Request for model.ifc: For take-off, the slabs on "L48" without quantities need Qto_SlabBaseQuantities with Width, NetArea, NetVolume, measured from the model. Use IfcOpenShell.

First a look at what the model holds.

```python
import ifcopenshell
import ifcopenshell.util.element
import ifcopenshell.util.unit

model = ifcopenshell.open("model.ifc")
print(model.schema)
for unit_type in ("LENGTHUNIT", "AREAUNIT", "VOLUMEUNIT"):
    print(unit_type, ifcopenshell.util.unit.calculate_unit_scale(model, unit_type))
storey = next(s for s in model.by_type("IfcBuildingStorey") if s.Name == "L48")
slabs = [e for e in ifcopenshell.util.element.get_decomposition(storey) if e.is_a("IfcSlab")]
for e in sorted(slabs, key=lambda e: e.id()):
    print(e.id(), e.is_a(), e.Name, list(ifcopenshell.util.element.get_psets(e, qtos_only=True)), sep=" | ")
```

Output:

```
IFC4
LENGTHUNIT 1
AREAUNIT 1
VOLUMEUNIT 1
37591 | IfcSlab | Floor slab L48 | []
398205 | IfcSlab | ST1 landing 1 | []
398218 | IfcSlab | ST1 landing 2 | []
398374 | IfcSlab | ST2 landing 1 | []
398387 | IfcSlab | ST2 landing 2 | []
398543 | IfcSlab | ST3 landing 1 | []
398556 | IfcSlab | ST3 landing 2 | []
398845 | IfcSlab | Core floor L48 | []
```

```python
import ifcopenshell
import ifcopenshell.api.pset
import ifcopenshell.geom
import ifcopenshell.util.element
import ifcopenshell.util.shape
import ifcopenshell.util.unit

model = ifcopenshell.open("model.ifc")
unit_scale = ifcopenshell.util.unit.calculate_unit_scale(model)
area_scale = ifcopenshell.util.unit.calculate_unit_scale(model, "AREAUNIT")
volume_scale = ifcopenshell.util.unit.calculate_unit_scale(model, "VOLUMEUNIT")
settings = ifcopenshell.geom.settings()

storey = next(s for s in model.by_type("IfcBuildingStorey") if s.Name == "L48")
slabs = [e for e in ifcopenshell.util.element.get_decomposition(storey) if e.is_a("IfcSlab")]

for e in sorted(slabs, key=lambda e: e.id()):
    if ifcopenshell.util.element.get_psets(e, qtos_only=True, should_inherit=False):
        continue
    # Geometry comes back in metres, in the element's own axes.
    shape = ifcopenshell.geom.create_shape(settings, e)
    values = {
        "Width": ifcopenshell.util.shape.get_z(shape.geometry) / unit_scale,
        "NetArea": ifcopenshell.util.shape.get_footprint_area(shape.geometry) / area_scale,
        "NetVolume": ifcopenshell.util.shape.get_volume(shape.geometry) / volume_scale,
    }
    qto = ifcopenshell.api.pset.add_qto(model, product=e, name="Qto_SlabBaseQuantities")
    ifcopenshell.api.pset.edit_qto(model, qto=qto, properties=values)
    print(e.id(), {k: round(v, 3) for k, v in values.items()})

model.write("model_rev.ifc")
```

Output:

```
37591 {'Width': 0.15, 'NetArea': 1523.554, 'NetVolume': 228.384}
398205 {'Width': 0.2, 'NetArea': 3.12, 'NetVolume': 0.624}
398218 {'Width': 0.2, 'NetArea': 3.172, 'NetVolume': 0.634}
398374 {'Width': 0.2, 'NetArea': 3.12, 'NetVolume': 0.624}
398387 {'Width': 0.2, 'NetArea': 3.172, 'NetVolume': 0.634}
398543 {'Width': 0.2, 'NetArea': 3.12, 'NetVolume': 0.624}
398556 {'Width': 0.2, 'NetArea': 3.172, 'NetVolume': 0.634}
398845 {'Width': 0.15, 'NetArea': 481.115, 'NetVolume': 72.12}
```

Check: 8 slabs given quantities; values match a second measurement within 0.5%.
